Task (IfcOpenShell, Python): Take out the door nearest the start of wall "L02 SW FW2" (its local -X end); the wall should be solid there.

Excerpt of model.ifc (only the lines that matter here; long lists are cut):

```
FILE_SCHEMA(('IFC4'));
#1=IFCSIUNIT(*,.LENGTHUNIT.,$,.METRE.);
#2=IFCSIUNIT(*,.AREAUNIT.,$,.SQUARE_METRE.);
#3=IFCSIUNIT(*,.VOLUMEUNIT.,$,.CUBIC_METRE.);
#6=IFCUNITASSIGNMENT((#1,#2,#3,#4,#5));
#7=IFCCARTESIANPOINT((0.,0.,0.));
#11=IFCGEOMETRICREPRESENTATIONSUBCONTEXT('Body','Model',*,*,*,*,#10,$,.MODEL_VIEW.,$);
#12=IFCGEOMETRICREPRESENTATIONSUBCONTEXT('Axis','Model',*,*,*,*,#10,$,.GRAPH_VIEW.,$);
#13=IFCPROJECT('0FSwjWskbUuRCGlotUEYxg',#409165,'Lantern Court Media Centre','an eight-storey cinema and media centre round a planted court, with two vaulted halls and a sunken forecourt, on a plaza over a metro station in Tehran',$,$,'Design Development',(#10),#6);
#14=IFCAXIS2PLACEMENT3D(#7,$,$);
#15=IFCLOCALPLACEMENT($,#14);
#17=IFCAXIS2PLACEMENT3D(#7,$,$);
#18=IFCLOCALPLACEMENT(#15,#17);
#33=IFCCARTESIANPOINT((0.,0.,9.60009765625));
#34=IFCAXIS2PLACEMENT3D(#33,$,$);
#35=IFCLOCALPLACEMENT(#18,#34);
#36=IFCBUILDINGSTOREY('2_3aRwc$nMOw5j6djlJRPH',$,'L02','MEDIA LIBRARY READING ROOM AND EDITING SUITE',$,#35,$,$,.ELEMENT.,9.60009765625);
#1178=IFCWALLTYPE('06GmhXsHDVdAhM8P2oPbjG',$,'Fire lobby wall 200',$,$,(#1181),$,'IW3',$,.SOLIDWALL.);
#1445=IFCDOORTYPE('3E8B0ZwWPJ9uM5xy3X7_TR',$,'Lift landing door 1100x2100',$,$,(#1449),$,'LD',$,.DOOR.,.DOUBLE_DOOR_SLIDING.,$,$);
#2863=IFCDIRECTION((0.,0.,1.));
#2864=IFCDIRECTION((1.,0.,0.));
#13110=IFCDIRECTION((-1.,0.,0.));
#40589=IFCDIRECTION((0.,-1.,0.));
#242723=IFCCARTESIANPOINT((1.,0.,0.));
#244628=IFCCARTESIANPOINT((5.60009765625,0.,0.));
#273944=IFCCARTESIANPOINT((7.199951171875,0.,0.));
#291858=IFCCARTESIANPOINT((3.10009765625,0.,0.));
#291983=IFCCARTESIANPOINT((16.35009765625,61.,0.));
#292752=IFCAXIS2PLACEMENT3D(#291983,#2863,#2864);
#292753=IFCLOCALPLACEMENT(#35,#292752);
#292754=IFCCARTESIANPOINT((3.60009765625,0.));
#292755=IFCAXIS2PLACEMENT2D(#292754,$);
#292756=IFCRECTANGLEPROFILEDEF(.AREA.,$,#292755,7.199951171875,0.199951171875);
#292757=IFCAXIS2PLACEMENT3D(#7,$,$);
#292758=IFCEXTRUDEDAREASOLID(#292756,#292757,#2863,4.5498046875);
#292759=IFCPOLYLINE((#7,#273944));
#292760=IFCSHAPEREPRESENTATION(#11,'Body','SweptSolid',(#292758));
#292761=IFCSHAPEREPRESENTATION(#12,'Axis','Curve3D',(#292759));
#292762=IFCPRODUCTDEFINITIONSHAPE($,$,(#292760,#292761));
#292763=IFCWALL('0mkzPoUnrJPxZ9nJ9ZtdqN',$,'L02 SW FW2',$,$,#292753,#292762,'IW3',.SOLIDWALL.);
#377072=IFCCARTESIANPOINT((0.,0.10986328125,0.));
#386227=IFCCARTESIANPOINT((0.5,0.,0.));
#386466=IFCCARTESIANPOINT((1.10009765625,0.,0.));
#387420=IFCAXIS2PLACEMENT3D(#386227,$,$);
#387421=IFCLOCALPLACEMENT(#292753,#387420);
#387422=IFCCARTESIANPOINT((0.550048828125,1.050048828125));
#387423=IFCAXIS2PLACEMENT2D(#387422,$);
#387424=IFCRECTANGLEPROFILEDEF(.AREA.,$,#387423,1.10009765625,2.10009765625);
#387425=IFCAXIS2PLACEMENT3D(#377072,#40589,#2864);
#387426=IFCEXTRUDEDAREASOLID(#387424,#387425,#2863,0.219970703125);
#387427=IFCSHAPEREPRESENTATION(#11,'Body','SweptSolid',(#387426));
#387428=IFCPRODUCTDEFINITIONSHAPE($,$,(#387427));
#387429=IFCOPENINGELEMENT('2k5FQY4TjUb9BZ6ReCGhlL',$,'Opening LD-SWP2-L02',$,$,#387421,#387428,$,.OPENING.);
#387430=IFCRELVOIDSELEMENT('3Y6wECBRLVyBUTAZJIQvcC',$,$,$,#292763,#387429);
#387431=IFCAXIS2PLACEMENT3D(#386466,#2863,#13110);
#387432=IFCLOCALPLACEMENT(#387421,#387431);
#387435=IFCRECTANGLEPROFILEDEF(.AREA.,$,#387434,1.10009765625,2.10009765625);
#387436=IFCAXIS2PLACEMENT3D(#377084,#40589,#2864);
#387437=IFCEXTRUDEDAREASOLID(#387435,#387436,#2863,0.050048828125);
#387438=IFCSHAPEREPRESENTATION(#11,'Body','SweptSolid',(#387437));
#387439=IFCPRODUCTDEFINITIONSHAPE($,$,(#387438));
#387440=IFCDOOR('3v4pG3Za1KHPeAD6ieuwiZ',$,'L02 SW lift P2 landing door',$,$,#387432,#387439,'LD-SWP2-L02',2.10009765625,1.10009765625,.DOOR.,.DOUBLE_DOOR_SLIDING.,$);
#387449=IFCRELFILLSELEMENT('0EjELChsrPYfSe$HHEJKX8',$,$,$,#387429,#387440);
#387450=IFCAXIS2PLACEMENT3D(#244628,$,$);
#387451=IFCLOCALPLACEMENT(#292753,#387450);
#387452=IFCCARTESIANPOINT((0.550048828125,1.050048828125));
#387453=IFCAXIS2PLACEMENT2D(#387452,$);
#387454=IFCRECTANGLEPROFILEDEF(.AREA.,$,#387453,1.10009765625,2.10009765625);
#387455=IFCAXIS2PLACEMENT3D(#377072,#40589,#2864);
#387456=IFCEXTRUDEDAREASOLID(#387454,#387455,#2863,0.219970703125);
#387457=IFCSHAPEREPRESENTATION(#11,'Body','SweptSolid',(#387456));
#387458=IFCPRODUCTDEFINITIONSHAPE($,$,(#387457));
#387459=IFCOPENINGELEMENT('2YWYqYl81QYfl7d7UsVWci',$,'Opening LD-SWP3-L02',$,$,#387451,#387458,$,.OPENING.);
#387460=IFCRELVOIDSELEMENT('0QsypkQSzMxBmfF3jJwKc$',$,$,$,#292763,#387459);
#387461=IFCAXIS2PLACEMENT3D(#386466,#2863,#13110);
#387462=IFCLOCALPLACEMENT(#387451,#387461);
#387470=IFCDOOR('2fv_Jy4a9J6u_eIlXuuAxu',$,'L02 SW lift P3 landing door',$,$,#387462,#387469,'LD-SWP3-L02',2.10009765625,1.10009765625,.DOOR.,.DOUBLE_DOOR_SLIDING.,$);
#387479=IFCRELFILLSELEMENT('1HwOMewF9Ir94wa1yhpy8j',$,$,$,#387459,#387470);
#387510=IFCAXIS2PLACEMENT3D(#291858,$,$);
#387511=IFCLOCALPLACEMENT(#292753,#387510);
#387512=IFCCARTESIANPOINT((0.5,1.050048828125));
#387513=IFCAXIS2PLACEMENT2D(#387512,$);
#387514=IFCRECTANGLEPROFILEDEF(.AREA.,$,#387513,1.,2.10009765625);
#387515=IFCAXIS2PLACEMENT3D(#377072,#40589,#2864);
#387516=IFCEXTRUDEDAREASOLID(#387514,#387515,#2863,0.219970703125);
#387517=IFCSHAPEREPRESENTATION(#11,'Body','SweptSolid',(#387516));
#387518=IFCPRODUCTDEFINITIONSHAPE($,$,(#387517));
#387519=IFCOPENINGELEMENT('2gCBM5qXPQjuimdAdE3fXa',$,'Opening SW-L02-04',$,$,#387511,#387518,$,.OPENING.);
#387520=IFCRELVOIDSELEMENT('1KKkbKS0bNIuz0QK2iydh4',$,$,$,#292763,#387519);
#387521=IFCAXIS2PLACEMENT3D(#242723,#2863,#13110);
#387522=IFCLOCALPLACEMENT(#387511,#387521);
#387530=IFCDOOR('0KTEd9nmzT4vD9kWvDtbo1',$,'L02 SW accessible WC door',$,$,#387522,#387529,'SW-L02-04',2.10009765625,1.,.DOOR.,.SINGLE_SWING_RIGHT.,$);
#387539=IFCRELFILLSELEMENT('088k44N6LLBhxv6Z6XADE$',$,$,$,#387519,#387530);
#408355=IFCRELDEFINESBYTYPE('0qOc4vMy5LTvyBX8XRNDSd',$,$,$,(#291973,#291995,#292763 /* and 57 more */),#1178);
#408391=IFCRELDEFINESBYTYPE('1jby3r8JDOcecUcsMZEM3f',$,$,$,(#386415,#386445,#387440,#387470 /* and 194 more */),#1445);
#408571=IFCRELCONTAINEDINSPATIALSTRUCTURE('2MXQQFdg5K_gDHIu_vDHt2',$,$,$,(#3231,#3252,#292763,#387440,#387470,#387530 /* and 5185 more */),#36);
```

```python
import ifcopenshell
import ifcopenshell.api.feature
import ifcopenshell.api.root
import ifcopenshell.geom
import ifcopenshell.util.shape

model = ifcopenshell.open("model.ifc")
settings = ifcopenshell.geom.settings()


def volume(element):
    """Net volume in cubic metres, openings subtracted."""
    shape = ifcopenshell.geom.create_shape(settings, element)
    return ifcopenshell.util.shape.get_volume(shape.geometry)


door = model.by_guid("3v4pG3Za1KHPeAD6ieuwiZ")
opening = door.FillsVoids[0].RelatingOpeningElement
wall = opening.VoidsElements[0].RelatingBuildingElement
before = volume(wall)

ifcopenshell.api.root.remove_product(model, product=door)
ifcopenshell.api.feature.remove_feature(model, feature=opening)

after = volume(wall)

print(f"wall volume {before:.3f} -> {after:.3f} m3")

model.write("model-out.ifc")
```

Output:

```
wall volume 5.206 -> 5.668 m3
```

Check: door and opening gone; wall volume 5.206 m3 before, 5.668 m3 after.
